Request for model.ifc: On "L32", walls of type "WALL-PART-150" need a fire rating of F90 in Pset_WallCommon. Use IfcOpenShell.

First a look at what the model holds.

```python
import ifcopenshell
import ifcopenshell.util.element

model = ifcopenshell.open("model.ifc")
print(model.schema)
storey = next(s for s in model.by_type("IfcBuildingStorey") if s.Name == "L32")
walls = [e for e in ifcopenshell.util.element.get_decomposition(storey) if e.is_a("IfcWall")]
seen = {}
for e in walls:
    element_type = ifcopenshell.util.element.get_type(e)
    key = (element_type.Name if element_type != e and element_type else None, ifcopenshell.util.element.get_pset(e, "Pset_WallCommon", "FireRating"))
    seen[key] = seen.get(key, 0) + 1
for (name, value), count in sorted(seen.items(), key=str):
    print(count, "x", name, "|", value)
```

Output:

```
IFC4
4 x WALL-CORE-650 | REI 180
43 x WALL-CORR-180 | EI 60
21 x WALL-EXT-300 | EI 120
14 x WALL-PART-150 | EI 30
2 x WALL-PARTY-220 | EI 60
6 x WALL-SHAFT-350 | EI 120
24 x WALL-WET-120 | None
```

```python
import ifcopenshell
import ifcopenshell.api.pset
import ifcopenshell.util.element

model = ifcopenshell.open("model.ifc")

storey = next(s for s in model.by_type("IfcBuildingStorey") if s.Name == "L32")
walls = [e for e in ifcopenshell.util.element.get_decomposition(storey) if e.is_a("IfcWall")]

count = 0
for e in walls:
    element_type = ifcopenshell.util.element.get_type(e)
    if element_type in (None, e) or element_type.Name != "WALL-PART-150":
        continue
    # add_pset returns the element's existing set when there is one.
    pset = ifcopenshell.api.pset.add_pset(model, product=e, name="Pset_WallCommon")
    ifcopenshell.api.pset.edit_pset(model, pset=pset, properties={"FireRating": "F90"})
    count += 1

print(count, "walls updated")

model.write("model_v2.ifc")
```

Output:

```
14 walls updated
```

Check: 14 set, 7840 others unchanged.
